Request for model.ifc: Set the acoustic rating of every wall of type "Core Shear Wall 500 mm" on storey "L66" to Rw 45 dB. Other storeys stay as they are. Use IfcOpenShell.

First a look at what the model holds.

```python
import ifcopenshell
import ifcopenshell.util.element

model = ifcopenshell.open("model.ifc")
print(model.schema)
storey = next(s for s in model.by_type("IfcBuildingStorey") if s.Name == "L66")
walls = [e for e in ifcopenshell.util.element.get_decomposition(storey) if e.is_a("IfcWall")]
seen = {}
for e in walls:
    element_type = ifcopenshell.util.element.get_type(e)
    key = (element_type.Name if element_type != e and element_type else None, ifcopenshell.util.element.get_pset(e, "Pset_WallCommon", "AcousticRating"))
    seen[key] = seen.get(key, 0) + 1
for (name, value), count in sorted(seen.items(), key=str):
    print(count, "x", name, "|", value)
```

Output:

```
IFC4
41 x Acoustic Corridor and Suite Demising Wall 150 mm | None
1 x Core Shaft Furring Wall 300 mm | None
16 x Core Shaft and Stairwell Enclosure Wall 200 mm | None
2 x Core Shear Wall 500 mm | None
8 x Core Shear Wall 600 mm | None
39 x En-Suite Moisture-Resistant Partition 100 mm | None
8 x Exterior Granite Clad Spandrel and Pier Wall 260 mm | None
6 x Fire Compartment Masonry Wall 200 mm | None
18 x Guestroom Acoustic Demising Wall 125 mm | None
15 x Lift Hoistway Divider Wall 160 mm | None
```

```python
import ifcopenshell
import ifcopenshell.api.pset
import ifcopenshell.util.element

model = ifcopenshell.open("model.ifc")

storey = next(s for s in model.by_type("IfcBuildingStorey") if s.Name == "L66")
walls = [e for e in ifcopenshell.util.element.get_decomposition(storey) if e.is_a("IfcWall")]

count = 0
for e in walls:
    element_type = ifcopenshell.util.element.get_type(e)
    if element_type in (None, e) or element_type.Name != "Core Shear Wall 500 mm":
        continue
    found = ifcopenshell.util.element.get_pset(e, "Pset_WallCommon", should_inherit=False)
    if found:
        pset = model.by_id(found["id"])
        if len(ifcopenshell.util.element.get_elements_by_pset(pset)) > 1:
            pset = ifcopenshell.api.pset.unshare_pset(model, products=[e], pset=pset)[0]
    else:
        pset = ifcopenshell.api.pset.add_pset(model, product=e, name="Pset_WallCommon")
    ifcopenshell.api.pset.edit_pset(model, pset=pset, properties={"AcousticRating": "Rw 45 dB"})
    count += 1

print(count, "walls updated")

model.write("model_rev.ifc")
```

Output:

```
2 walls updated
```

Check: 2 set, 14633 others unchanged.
